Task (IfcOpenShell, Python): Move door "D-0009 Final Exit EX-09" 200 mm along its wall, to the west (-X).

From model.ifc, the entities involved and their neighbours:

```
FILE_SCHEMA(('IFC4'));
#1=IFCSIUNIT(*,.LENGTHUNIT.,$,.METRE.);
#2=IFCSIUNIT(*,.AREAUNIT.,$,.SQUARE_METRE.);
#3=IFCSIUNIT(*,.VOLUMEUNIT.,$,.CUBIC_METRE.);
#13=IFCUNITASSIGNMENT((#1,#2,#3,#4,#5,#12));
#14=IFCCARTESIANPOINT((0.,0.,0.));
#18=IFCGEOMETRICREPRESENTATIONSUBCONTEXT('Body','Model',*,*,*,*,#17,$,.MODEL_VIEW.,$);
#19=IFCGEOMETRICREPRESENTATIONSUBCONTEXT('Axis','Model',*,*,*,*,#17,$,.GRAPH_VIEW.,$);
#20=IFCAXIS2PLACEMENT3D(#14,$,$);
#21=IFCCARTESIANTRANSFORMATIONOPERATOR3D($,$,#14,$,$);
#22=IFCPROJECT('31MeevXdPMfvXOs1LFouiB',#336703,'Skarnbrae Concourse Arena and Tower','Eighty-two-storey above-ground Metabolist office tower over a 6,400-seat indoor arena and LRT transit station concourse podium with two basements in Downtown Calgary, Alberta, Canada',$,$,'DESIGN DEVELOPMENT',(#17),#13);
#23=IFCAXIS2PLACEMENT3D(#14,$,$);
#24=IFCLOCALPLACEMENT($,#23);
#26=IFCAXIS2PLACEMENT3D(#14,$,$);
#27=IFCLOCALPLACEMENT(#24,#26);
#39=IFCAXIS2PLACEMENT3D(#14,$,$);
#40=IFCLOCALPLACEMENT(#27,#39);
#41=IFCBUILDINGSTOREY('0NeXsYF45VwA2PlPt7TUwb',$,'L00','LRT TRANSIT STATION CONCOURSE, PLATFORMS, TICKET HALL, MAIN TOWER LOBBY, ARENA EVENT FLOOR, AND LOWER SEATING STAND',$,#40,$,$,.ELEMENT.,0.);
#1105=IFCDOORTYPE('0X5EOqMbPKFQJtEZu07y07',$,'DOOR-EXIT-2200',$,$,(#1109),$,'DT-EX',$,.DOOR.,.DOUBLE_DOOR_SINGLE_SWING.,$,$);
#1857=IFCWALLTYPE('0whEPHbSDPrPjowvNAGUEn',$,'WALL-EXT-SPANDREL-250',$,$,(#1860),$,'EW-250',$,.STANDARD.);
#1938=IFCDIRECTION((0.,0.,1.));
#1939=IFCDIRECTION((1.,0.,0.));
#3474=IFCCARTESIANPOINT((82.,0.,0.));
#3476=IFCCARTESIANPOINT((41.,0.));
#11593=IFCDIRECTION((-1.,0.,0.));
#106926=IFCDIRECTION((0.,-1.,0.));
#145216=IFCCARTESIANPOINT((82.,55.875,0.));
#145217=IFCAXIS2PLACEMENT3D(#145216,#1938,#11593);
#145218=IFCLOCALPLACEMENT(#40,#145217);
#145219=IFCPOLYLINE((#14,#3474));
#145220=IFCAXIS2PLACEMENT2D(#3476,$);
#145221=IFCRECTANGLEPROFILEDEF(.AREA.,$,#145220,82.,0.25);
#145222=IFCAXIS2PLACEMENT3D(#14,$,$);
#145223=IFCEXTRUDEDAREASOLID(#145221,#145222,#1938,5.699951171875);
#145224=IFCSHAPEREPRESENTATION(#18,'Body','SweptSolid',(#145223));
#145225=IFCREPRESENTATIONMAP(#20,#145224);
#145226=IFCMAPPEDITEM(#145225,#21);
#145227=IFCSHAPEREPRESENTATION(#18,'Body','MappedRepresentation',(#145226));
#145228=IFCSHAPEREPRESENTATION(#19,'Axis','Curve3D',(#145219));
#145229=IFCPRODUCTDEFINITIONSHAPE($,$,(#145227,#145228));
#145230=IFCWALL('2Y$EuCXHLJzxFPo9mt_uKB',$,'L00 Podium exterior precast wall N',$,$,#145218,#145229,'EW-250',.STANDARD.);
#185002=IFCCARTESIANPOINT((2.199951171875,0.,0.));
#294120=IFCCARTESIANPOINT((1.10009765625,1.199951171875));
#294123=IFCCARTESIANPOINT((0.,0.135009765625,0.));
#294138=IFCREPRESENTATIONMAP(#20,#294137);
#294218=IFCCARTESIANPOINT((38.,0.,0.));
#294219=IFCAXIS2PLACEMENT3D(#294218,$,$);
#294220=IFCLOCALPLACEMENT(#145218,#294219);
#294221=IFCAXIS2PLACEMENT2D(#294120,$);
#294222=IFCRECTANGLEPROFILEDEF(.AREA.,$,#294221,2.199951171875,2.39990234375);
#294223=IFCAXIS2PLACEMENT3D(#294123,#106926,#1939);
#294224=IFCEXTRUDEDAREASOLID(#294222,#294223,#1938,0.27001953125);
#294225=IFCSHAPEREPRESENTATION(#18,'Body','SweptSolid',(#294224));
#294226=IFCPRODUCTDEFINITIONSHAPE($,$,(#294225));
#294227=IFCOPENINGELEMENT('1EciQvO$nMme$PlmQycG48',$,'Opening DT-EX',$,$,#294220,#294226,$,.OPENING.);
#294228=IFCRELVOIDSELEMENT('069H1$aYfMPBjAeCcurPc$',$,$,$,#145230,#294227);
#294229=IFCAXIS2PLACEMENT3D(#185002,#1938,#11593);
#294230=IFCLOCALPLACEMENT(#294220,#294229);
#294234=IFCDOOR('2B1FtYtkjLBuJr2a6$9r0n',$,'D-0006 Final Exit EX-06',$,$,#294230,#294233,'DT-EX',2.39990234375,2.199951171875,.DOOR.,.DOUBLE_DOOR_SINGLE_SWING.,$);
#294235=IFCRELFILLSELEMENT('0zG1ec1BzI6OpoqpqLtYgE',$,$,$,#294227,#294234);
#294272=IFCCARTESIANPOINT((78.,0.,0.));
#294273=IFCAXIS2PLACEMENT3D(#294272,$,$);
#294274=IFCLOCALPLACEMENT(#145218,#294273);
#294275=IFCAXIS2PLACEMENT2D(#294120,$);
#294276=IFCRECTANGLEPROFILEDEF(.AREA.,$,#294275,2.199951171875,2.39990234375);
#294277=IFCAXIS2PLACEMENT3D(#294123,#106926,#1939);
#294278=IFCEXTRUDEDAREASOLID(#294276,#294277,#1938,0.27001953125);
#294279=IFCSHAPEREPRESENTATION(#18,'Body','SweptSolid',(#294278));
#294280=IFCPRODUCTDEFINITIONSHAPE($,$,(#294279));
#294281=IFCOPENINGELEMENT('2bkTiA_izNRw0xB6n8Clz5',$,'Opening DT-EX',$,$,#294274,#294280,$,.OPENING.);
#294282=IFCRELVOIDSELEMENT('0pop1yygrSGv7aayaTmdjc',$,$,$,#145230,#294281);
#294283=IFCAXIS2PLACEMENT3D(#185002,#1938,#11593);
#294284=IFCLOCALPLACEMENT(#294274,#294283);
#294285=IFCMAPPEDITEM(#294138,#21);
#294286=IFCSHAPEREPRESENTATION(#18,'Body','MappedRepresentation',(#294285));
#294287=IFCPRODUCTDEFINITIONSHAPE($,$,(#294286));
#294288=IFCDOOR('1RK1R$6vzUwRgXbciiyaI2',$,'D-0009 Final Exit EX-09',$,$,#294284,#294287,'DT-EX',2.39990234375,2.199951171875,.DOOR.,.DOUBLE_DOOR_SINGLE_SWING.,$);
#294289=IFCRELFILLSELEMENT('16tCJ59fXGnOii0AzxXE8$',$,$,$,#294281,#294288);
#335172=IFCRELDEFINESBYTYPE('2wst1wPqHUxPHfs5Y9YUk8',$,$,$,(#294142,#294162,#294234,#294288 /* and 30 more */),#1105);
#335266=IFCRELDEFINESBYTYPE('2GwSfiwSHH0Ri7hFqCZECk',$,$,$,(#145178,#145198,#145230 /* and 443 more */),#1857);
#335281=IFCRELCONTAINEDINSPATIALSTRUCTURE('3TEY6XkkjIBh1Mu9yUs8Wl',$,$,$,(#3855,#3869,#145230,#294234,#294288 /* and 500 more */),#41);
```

```python
import ifcopenshell
import ifcopenshell.api.geometry
import ifcopenshell.util.placement
import ifcopenshell.util.unit

model = ifcopenshell.open("model.ifc")
unit_scale = ifcopenshell.util.unit.calculate_unit_scale(model)

door = model.by_guid("1RK1R$6vzUwRgXbciiyaI2")
opening = door.FillsVoids[0].RelatingOpeningElement
wall = opening.VoidsElements[0].RelatingBuildingElement

wall_matrix = ifcopenshell.util.placement.get_local_placement(wall.ObjectPlacement)
shift = wall_matrix[:3, 0] * 0.2 / unit_scale
before = ifcopenshell.util.placement.get_local_placement(door.ObjectPlacement)[:3, 3].copy()

# The door is placed relative to its opening, so it follows when the opening moves.
matrix = ifcopenshell.util.placement.get_local_placement(opening.ObjectPlacement)
matrix[:3, 3] += shift
ifcopenshell.api.geometry.edit_object_placement(
    model, product=opening, matrix=matrix, is_si=False, should_transform_children=True
)

after = ifcopenshell.util.placement.get_local_placement(door.ObjectPlacement)[:3, 3]
print("door moved by", (after - before).round(3) + 0.0)

model.write("model-out.ifc")
```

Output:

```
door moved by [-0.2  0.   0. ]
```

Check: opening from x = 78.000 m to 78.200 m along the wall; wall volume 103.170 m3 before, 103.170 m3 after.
